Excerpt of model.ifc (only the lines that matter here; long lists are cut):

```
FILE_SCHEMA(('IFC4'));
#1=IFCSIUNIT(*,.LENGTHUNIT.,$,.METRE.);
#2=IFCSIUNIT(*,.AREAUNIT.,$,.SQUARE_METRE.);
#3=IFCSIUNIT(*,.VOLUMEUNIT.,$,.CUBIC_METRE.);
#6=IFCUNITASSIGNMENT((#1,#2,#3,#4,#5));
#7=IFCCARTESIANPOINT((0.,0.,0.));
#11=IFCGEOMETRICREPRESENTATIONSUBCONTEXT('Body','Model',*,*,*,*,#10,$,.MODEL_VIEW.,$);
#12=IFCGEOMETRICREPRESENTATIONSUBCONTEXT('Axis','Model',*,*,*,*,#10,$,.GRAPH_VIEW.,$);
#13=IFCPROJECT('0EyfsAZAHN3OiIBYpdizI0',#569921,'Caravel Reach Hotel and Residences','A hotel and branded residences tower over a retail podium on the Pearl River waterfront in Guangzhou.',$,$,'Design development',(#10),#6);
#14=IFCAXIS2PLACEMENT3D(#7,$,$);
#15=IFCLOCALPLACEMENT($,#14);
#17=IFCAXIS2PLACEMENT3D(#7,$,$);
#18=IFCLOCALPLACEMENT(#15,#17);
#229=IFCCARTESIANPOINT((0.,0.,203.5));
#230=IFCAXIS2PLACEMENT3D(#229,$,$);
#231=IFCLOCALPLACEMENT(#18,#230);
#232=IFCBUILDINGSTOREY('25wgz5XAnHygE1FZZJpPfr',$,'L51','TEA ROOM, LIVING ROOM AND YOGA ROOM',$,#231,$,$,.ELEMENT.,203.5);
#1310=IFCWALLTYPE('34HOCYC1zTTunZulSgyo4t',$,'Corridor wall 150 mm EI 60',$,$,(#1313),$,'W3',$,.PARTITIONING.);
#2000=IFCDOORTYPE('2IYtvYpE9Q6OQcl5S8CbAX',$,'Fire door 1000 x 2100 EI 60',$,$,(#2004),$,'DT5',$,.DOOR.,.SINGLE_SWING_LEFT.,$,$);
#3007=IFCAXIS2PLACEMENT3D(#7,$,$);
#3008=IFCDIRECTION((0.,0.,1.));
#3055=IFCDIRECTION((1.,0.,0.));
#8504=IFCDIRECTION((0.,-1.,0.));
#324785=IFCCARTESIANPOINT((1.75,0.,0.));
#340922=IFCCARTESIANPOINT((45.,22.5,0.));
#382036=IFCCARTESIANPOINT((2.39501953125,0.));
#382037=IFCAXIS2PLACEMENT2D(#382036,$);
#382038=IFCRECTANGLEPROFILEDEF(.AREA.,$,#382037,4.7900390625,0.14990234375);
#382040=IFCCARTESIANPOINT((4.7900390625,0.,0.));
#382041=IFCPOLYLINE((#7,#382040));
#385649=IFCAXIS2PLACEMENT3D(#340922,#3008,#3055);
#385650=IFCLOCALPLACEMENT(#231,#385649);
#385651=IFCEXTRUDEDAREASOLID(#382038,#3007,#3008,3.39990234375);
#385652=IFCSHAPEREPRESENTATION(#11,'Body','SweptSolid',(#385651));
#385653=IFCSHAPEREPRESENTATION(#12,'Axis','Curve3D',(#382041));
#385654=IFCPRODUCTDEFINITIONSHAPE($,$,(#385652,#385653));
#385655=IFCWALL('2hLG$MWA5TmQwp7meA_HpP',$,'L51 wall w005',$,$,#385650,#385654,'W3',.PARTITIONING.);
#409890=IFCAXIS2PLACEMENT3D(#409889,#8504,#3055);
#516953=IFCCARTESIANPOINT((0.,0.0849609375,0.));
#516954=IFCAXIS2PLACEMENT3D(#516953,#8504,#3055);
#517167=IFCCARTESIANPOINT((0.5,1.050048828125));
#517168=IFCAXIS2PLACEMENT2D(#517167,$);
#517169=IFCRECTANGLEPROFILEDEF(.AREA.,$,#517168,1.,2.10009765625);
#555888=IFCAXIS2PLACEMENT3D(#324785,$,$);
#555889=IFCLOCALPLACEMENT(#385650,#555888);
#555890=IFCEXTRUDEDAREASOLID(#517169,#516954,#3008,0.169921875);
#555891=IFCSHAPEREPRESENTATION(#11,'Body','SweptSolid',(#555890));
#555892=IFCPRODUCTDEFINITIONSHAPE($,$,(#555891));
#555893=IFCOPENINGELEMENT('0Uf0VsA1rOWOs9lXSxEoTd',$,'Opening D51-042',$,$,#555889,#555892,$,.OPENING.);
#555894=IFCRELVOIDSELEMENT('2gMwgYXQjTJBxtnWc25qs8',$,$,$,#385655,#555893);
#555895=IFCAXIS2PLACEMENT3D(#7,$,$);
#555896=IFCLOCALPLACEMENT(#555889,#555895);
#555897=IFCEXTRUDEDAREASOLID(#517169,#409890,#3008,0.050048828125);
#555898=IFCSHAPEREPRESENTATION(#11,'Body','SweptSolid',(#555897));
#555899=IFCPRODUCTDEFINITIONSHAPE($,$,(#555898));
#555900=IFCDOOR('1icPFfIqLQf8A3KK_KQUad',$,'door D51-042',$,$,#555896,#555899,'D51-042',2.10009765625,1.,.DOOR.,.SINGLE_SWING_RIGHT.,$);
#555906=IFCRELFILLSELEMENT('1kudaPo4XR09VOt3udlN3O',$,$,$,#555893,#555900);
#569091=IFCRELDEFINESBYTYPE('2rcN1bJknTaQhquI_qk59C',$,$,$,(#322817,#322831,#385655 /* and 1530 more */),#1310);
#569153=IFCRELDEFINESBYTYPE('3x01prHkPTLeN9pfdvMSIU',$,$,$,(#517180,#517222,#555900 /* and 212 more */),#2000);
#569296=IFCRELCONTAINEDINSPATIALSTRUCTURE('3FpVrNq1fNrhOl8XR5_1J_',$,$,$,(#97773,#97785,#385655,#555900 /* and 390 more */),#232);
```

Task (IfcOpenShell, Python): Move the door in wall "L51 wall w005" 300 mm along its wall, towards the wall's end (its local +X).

```python
import ifcopenshell
import ifcopenshell.api.geometry
import ifcopenshell.util.placement
import ifcopenshell.util.unit

model = ifcopenshell.open("model.ifc")
unit_scale = ifcopenshell.util.unit.calculate_unit_scale(model)

door = model.by_guid("1icPFfIqLQf8A3KK_KQUad")
opening = door.FillsVoids[0].RelatingOpeningElement
wall = opening.VoidsElements[0].RelatingBuildingElement

wall_matrix = ifcopenshell.util.placement.get_local_placement(wall.ObjectPlacement)
shift = wall_matrix[:3, 0] * 0.3 / unit_scale
before = ifcopenshell.util.placement.get_local_placement(door.ObjectPlacement)[:3, 3].copy()

# The door is placed relative to its opening, so it follows when the opening moves.
matrix = ifcopenshell.util.placement.get_local_placement(opening.ObjectPlacement)
matrix[:3, 3] += shift
ifcopenshell.api.geometry.edit_object_placement(
    model, product=opening, matrix=matrix, is_si=False, should_transform_children=True
)

after = ifcopenshell.util.placement.get_local_placement(door.ObjectPlacement)[:3, 3]
print("door moved by", (after - before).round(3) + 0.0)

model.write("model_rev.ifc")
```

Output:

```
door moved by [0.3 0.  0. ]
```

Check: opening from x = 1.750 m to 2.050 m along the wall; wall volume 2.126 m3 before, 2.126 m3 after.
